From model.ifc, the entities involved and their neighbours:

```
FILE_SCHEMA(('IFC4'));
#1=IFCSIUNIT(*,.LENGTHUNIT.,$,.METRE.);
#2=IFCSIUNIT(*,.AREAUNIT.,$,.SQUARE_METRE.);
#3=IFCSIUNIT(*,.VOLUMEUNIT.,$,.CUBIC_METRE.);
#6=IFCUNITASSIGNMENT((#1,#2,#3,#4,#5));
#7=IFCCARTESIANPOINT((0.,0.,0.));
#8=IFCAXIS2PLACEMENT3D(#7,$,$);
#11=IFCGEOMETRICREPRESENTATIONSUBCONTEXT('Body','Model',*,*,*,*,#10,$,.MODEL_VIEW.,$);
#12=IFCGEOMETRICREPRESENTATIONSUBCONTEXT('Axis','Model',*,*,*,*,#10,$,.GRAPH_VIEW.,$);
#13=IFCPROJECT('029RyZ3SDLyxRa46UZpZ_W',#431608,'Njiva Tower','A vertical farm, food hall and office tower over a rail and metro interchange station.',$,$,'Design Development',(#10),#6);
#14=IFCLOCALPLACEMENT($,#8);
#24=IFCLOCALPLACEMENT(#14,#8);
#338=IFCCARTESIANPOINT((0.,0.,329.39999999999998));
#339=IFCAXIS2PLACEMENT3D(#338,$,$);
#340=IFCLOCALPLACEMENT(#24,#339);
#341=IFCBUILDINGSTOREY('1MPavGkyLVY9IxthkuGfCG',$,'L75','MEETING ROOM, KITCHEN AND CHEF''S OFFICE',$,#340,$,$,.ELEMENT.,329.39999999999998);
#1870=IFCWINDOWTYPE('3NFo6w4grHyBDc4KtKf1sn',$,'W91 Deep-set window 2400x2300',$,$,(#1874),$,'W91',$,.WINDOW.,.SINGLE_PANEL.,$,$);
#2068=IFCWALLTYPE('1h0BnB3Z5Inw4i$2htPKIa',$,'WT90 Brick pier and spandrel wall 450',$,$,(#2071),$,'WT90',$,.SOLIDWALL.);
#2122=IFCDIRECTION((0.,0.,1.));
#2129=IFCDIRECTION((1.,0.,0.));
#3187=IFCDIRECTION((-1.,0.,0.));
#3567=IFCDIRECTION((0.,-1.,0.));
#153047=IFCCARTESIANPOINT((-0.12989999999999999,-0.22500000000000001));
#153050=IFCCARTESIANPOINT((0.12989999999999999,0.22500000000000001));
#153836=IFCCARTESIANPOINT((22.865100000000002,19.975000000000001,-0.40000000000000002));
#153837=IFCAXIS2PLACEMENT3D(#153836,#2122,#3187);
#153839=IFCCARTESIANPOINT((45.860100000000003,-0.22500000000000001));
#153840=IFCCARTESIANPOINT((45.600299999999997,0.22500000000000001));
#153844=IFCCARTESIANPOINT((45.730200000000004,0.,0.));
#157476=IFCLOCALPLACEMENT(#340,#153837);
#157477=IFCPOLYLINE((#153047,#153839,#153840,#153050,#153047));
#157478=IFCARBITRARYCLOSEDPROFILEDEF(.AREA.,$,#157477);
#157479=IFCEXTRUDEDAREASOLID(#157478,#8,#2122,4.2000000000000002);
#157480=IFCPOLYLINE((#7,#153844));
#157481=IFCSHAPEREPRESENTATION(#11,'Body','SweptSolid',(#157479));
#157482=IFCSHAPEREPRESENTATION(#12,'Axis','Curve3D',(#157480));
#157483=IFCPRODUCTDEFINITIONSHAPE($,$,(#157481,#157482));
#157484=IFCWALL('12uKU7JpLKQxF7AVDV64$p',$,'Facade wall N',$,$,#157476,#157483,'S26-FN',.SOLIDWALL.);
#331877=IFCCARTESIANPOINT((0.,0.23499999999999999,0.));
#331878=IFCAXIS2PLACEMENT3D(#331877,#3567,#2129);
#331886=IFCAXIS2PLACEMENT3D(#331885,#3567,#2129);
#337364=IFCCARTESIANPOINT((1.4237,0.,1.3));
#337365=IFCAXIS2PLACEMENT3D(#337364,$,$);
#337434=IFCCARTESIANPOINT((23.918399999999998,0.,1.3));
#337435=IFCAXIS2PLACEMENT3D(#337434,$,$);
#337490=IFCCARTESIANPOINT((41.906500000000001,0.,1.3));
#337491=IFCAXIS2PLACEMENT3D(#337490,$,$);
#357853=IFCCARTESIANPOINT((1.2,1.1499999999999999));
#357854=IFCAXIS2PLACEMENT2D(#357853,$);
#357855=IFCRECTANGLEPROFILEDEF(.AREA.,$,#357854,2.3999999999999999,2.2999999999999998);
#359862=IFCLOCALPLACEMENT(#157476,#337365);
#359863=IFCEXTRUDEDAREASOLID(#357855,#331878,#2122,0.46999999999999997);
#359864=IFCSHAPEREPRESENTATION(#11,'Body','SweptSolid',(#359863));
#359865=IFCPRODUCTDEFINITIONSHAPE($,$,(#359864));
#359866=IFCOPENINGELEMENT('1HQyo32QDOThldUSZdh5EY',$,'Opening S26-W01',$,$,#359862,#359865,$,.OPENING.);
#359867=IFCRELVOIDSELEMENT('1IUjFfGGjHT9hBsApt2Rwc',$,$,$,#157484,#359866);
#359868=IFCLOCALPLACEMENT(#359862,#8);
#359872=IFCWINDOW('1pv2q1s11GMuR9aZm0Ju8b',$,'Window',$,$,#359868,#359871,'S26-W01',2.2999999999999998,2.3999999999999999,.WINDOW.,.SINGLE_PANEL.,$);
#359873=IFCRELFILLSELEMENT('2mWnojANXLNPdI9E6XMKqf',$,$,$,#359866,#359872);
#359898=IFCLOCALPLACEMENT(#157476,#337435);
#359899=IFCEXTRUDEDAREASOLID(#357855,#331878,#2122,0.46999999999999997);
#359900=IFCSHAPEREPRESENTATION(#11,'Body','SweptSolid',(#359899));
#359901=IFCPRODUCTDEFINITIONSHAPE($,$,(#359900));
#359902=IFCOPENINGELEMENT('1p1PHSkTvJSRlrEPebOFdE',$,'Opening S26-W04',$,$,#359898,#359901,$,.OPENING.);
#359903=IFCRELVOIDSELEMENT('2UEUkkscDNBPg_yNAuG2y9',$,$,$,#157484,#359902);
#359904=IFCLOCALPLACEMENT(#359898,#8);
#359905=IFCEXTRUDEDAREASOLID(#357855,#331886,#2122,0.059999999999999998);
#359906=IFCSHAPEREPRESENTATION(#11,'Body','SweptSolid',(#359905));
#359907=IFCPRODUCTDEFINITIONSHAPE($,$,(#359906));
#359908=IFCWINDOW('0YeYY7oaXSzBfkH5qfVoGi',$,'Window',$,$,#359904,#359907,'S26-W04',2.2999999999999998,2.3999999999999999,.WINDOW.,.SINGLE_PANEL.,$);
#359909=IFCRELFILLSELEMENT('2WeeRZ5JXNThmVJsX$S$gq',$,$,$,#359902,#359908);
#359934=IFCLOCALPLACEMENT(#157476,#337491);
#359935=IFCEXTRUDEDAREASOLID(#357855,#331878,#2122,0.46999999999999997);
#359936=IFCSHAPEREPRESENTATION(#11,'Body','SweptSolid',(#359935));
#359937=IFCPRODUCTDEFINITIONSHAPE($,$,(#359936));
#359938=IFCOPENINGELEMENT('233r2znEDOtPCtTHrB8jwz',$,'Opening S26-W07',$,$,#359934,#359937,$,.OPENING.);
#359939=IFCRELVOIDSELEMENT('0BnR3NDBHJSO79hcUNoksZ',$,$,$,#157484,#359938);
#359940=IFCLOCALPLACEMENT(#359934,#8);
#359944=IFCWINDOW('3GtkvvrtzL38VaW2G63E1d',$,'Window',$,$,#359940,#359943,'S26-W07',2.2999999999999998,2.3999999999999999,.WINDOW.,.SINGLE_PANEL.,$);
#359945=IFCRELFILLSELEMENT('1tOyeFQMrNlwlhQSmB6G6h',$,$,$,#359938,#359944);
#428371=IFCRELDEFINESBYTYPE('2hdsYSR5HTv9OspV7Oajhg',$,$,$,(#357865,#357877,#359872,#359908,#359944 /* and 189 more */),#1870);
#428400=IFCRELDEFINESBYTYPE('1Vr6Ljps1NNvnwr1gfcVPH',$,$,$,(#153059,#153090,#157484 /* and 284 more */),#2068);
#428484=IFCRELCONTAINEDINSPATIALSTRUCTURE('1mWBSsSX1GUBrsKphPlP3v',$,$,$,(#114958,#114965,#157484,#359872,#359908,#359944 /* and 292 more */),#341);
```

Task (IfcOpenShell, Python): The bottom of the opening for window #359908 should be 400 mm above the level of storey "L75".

```python
import numpy as np
import ifcopenshell
import ifcopenshell.api.geometry
import ifcopenshell.geom
import ifcopenshell.util.element
import ifcopenshell.util.placement
import ifcopenshell.util.shape
import ifcopenshell.util.unit

model = ifcopenshell.open("model.ifc")
unit_scale = ifcopenshell.util.unit.calculate_unit_scale(model)

window = model.by_id(359908)
opening = window.FillsVoids[0].RelatingOpeningElement
storey = ifcopenshell.util.element.get_container(window, ifc_class="IfcBuildingStorey")
level = ifcopenshell.util.placement.get_local_placement(storey.ObjectPlacement)[2, 3]

# The opening's origin need not be at the sill, so measure its lowest point.
shape = ifcopenshell.geom.create_shape(ifcopenshell.geom.settings(), opening)
bottom = ifcopenshell.util.shape.get_shape_bottom_elevation(shape, shape.geometry) / unit_scale
dz = level + 0.4 / unit_scale - bottom

shift = np.array([0.0, 0.0, dz])
# The window is placed relative to its opening, so it follows when the opening moves.
matrix = ifcopenshell.util.placement.get_local_placement(opening.ObjectPlacement)
matrix[:3, 3] += shift
ifcopenshell.api.geometry.edit_object_placement(
    model, product=opening, matrix=matrix, is_si=False, should_transform_children=True
)

print(f"moved by {dz * unit_scale:+.3f} m")

model.write("model-out.ifc")
```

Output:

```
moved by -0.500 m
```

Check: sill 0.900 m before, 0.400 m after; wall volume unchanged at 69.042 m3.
